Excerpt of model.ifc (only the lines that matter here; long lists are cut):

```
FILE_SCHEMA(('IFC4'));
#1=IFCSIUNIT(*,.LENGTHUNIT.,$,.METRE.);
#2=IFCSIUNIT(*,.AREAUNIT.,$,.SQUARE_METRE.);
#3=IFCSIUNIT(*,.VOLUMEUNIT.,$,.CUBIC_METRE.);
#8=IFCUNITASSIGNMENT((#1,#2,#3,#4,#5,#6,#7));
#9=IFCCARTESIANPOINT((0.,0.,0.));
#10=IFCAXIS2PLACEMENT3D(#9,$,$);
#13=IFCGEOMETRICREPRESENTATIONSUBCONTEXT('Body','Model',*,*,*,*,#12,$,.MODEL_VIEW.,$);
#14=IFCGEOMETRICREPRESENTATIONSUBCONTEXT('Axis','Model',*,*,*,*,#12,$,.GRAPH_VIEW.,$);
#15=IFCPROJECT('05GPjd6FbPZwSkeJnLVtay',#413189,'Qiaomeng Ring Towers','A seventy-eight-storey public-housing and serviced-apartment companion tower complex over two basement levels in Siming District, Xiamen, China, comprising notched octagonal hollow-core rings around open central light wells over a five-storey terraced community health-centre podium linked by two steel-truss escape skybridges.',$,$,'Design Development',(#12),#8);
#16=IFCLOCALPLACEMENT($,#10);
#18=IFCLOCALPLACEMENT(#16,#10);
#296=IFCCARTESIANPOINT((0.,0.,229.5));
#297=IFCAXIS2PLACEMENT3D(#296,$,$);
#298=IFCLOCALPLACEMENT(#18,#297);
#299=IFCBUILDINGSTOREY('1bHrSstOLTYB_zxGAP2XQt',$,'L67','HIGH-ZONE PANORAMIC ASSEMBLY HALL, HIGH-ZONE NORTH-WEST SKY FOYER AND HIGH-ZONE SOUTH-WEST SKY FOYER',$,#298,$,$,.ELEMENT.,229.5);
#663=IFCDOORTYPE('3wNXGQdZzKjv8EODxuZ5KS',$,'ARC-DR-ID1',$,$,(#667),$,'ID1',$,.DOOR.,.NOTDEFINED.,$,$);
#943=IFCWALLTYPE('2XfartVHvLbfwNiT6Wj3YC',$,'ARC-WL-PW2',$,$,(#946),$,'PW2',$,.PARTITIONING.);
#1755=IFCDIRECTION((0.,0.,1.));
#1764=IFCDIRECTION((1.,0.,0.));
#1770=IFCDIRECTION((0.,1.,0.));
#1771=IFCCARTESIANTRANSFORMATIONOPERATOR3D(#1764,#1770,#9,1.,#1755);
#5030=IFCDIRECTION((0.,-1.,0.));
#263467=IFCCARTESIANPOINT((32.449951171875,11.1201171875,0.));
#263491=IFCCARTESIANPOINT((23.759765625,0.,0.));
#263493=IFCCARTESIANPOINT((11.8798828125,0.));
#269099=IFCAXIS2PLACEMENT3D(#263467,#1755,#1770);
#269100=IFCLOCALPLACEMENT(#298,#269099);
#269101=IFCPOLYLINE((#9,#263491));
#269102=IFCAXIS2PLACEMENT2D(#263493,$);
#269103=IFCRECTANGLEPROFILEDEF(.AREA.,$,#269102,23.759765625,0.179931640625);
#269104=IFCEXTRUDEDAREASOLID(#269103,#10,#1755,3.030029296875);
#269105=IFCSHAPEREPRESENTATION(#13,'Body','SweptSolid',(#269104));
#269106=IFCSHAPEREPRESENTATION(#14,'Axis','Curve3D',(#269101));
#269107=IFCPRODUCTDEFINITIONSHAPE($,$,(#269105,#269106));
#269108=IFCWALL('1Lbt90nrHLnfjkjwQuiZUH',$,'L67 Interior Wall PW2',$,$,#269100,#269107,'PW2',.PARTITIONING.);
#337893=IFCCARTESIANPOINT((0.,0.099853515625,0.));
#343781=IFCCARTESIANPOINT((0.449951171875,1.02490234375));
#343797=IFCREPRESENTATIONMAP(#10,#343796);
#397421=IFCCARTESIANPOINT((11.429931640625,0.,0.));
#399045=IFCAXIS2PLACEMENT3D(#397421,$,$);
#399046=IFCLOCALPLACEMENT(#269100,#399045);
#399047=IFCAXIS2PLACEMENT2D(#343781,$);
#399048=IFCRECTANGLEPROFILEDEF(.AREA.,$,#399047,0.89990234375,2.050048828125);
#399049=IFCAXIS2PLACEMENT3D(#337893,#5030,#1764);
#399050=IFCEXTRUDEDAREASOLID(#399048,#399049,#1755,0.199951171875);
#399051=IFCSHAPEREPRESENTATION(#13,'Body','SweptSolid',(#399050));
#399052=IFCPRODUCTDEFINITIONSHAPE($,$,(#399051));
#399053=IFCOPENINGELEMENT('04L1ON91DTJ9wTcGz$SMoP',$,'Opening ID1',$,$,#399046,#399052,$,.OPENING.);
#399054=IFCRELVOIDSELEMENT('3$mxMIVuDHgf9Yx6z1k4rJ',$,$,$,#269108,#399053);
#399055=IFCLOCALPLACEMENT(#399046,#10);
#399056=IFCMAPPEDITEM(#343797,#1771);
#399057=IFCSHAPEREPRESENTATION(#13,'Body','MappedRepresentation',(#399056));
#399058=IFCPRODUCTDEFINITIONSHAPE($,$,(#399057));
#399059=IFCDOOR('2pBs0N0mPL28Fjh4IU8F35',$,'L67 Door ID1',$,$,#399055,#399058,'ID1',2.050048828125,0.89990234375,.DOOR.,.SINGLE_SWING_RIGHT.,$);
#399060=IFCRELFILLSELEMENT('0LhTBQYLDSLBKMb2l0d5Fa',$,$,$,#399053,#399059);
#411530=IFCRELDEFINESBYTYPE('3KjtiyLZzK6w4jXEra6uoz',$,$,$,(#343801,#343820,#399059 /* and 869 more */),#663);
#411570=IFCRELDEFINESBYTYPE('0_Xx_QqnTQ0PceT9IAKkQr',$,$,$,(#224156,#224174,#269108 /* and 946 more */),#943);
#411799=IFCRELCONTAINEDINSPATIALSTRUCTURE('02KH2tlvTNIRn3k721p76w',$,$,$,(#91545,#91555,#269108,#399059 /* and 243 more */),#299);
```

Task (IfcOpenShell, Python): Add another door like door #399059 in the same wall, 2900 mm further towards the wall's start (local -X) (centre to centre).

```python
import ifcopenshell
import ifcopenshell.api.feature
import ifcopenshell.api.geometry
import ifcopenshell.api.root
import ifcopenshell.geom
import ifcopenshell.util.element
import ifcopenshell.util.placement
import ifcopenshell.util.shape
import ifcopenshell.util.unit

model = ifcopenshell.open("model.ifc")
unit_scale = ifcopenshell.util.unit.calculate_unit_scale(model)
settings = ifcopenshell.geom.settings()


def volume(element):
    """Net volume in cubic metres, openings subtracted."""
    shape = ifcopenshell.geom.create_shape(settings, element)
    return ifcopenshell.util.shape.get_volume(shape.geometry)


door = model.by_guid("2pBs0N0mPL28Fjh4IU8F35")
opening = door.FillsVoids[0].RelatingOpeningElement
wall = opening.VoidsElements[0].RelatingBuildingElement
before = volume(wall)
shift = ifcopenshell.util.placement.get_local_placement(wall.ObjectPlacement)[:3, 0] * -2.9 / unit_scale

# copy_class copies the void relationship, type, container and properties, but no geometry.
new_opening = ifcopenshell.api.root.copy_class(model, product=opening)
new_opening.Representation = ifcopenshell.util.element.copy_deep(
    model, opening.Representation, exclude=["IfcGeometricRepresentationContext", "IfcRepresentationMap"]
)
new_door = ifcopenshell.api.root.copy_class(model, product=door)
new_door.Representation = ifcopenshell.util.element.copy_deep(
    model, door.Representation, exclude=["IfcGeometricRepresentationContext", "IfcRepresentationMap"]
)
new_door.Tag = None
ifcopenshell.api.feature.add_filling(model, opening=new_opening, element=new_door)

for old, new in ((opening, new_opening), (door, new_door)):
    matrix = ifcopenshell.util.placement.get_local_placement(old.ObjectPlacement)
    matrix[:3, 3] += shift
    ifcopenshell.api.geometry.edit_object_placement(model, product=new, matrix=matrix, is_si=False)

after = volume(wall)

print(f"wall volume {before:.3f} -> {after:.3f} m3")

model.write("model_updated.ifc")
```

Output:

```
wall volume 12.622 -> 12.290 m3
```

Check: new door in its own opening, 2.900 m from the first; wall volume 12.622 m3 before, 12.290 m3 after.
